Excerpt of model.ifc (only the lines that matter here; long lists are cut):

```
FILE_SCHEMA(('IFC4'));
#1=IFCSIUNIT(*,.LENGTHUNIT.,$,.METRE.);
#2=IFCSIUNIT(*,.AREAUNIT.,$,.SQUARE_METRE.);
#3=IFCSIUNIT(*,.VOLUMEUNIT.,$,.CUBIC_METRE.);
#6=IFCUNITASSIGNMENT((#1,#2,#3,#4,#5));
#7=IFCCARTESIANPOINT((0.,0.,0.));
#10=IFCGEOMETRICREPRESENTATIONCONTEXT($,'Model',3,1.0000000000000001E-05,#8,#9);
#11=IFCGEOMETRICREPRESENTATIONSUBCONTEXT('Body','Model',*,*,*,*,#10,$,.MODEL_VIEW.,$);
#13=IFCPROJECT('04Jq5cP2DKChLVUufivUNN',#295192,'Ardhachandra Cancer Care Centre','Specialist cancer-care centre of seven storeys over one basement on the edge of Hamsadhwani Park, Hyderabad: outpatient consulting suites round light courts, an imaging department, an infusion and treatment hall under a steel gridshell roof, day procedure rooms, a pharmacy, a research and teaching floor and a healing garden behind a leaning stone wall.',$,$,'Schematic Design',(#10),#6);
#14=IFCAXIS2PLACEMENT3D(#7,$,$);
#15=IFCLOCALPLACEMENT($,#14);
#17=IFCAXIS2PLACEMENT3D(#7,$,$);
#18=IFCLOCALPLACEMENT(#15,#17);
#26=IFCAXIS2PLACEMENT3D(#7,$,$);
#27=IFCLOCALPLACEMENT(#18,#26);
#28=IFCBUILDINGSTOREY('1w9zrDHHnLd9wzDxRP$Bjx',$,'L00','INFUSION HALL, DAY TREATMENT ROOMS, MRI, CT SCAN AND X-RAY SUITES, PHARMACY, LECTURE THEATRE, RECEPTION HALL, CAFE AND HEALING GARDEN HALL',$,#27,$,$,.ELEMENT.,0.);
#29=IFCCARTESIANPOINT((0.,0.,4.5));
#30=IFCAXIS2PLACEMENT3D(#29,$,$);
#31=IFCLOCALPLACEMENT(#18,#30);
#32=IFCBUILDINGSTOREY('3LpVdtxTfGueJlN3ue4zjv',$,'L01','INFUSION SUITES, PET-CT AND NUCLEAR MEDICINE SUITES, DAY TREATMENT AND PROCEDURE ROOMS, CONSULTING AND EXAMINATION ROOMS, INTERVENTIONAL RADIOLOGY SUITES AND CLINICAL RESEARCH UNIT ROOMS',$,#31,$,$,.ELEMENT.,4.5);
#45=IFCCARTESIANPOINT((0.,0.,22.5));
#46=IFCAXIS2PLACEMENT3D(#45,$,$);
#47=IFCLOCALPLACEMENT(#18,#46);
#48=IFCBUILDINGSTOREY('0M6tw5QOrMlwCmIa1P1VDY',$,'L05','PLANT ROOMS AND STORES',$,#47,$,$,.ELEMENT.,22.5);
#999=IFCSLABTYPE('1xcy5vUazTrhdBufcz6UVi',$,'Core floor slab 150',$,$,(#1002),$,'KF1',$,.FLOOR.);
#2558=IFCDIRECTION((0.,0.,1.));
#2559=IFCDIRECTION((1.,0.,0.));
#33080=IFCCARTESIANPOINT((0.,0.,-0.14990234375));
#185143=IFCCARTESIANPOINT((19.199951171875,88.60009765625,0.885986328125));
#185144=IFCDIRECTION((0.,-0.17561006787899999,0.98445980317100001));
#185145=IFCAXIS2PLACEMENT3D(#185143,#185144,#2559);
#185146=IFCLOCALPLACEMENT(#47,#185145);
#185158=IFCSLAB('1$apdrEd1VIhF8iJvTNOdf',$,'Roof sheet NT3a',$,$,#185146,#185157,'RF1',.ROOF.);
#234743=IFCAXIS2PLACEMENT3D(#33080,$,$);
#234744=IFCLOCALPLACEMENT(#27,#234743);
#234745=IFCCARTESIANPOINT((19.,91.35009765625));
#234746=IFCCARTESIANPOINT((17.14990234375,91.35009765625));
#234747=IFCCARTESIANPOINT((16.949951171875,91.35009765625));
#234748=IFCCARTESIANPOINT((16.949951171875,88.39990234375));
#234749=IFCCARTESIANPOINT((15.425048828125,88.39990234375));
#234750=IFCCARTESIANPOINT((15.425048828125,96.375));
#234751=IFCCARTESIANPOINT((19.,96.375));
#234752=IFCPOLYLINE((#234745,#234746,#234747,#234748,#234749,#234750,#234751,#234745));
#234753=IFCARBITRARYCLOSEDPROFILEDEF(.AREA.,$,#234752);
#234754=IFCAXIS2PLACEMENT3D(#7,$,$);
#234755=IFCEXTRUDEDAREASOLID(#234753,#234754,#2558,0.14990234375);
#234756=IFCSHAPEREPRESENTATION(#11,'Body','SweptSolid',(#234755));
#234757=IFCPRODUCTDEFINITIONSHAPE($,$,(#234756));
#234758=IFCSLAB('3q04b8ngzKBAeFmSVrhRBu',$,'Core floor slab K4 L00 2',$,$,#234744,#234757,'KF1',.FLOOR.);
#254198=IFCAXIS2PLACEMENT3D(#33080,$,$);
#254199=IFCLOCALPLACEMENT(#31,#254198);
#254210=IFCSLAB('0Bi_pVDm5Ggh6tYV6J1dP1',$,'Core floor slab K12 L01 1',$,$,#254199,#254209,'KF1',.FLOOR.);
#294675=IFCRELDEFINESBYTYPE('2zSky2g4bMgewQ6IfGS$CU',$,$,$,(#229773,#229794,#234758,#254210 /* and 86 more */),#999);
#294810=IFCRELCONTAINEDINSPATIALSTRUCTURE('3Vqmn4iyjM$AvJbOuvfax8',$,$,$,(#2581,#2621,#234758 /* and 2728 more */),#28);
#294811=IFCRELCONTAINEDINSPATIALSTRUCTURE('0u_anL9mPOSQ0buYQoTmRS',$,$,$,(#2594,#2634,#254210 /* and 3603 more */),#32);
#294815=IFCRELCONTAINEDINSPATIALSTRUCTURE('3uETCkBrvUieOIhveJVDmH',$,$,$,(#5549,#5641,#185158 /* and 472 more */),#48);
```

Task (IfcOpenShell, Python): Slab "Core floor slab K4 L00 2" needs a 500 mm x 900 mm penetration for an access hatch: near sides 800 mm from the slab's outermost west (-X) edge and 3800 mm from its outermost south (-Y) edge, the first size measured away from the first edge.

```python
import numpy as np
import ifcopenshell
import ifcopenshell.api.feature
import ifcopenshell.api.geometry
import ifcopenshell.api.root
import ifcopenshell.geom
import ifcopenshell.util.placement
import ifcopenshell.util.representation
import ifcopenshell.util.shape
import ifcopenshell.util.unit

model = ifcopenshell.open("model.ifc")
unit_scale = ifcopenshell.util.unit.calculate_unit_scale(model)
settings = ifcopenshell.geom.settings()


def volume(element):
    """Net volume in cubic metres, openings subtracted."""
    shape = ifcopenshell.geom.create_shape(settings, element)
    return ifcopenshell.util.shape.get_volume(shape.geometry)


slab = model.by_guid("3q04b8ngzKBAeFmSVrhRBu")
before = volume(slab)

# Extent in the slab's own axes, in metres. The edges named are its -X and -Y sides.
slab_shape = ifcopenshell.geom.create_shape(settings, slab)
vertices = ifcopenshell.util.shape.get_vertices(slab_shape.geometry)
x_min, y_min, bottom = vertices.min(axis=0)
top = vertices[:, 2].max()

opening = ifcopenshell.api.root.create_entity(model, ifc_class="IfcOpeningElement", name="Access hatch opening", predefined_type="OPENING")
context = ifcopenshell.util.representation.get_context(model, "Model", "Body", "MODEL_VIEW")
width, depth = 0.5, 0.9
outline = [(0.0, 0.0), (width, 0.0), (width, depth), (0.0, depth), (0.0, 0.0)]
# Overshoot both faces by 50 mm so the cut is clean.
shape = ifcopenshell.api.geometry.add_slab_representation(
    model, context=context, depth=top - bottom + 0.1, polyline=outline
)
ifcopenshell.api.geometry.assign_representation(model, product=opening, representation=shape)

matrix = ifcopenshell.util.placement.get_local_placement(slab.ObjectPlacement)
matrix[:, 3] = matrix @ np.append(np.array([x_min + 0.8, y_min + 3.8, bottom - 0.05]) / unit_scale, 1.0)
ifcopenshell.api.geometry.edit_object_placement(model, product=opening, matrix=matrix, is_si=False)
ifcopenshell.api.feature.add_feature(model, feature=opening, element=slab)

after = volume(slab)

print(f"slab volume {before:.3f} -> {after:.3f} m3")

model.write("model_rev.ifc")
```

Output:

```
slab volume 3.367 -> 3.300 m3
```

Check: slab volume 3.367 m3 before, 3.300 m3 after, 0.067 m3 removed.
